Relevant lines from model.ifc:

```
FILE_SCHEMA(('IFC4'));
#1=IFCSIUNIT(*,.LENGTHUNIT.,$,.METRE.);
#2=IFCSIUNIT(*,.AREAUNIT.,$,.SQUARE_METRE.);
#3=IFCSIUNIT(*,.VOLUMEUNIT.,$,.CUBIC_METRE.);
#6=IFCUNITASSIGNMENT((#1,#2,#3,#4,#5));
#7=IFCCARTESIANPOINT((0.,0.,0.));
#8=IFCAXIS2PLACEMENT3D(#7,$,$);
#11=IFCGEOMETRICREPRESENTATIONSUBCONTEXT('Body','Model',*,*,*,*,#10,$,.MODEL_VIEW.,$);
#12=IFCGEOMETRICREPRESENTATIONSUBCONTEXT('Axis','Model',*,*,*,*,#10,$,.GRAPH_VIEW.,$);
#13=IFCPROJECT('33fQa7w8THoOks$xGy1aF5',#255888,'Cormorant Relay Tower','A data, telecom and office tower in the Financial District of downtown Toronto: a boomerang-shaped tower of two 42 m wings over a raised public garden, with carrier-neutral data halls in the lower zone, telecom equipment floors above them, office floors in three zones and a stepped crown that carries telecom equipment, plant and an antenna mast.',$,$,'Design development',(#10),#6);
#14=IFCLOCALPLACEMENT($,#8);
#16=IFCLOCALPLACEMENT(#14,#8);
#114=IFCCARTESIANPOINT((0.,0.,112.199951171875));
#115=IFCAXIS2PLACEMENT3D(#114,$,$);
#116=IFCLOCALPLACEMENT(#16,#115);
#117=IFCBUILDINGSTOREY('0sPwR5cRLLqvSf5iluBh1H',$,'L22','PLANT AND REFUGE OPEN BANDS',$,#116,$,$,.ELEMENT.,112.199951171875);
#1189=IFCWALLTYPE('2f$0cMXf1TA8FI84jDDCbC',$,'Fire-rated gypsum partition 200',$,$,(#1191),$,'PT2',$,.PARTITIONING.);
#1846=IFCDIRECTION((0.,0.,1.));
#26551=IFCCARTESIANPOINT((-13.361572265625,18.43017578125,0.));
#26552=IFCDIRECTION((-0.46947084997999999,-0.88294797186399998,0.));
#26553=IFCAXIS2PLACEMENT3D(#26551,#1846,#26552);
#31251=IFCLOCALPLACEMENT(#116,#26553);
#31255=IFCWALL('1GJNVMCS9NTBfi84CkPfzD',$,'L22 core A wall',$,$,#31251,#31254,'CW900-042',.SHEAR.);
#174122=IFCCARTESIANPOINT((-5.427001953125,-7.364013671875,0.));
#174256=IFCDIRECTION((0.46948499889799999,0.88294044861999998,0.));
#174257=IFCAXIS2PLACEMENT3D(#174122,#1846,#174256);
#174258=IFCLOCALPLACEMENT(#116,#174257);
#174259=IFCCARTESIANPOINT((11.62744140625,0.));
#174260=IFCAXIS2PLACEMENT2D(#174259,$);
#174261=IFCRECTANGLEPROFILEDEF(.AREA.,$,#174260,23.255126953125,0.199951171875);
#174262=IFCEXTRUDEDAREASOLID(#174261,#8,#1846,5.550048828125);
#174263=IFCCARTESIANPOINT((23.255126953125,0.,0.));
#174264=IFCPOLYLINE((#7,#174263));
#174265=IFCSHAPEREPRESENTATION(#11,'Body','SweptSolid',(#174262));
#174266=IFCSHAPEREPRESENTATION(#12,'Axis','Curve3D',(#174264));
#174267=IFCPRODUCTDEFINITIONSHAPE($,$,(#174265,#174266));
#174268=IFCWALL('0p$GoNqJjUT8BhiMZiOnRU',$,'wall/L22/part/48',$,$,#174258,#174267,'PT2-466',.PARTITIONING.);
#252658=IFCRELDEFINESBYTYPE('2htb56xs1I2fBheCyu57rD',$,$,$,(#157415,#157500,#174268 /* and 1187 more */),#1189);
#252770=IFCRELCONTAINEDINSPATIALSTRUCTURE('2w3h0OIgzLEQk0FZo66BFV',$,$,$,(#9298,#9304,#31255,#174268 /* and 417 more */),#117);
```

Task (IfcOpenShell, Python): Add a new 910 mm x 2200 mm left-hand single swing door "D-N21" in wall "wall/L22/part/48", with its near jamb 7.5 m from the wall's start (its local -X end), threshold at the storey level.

```python
import numpy as np
import ifcopenshell
import ifcopenshell.api.feature
import ifcopenshell.api.geometry
import ifcopenshell.api.root
import ifcopenshell.api.spatial
import ifcopenshell.geom
import ifcopenshell.util.element
import ifcopenshell.util.placement
import ifcopenshell.util.representation
import ifcopenshell.util.shape
import ifcopenshell.util.unit

model = ifcopenshell.open("model.ifc")
unit_scale = ifcopenshell.util.unit.calculate_unit_scale(model)
settings = ifcopenshell.geom.settings()


def volume(element):
    """Net volume in cubic metres, openings subtracted."""
    shape = ifcopenshell.geom.create_shape(settings, element)
    return ifcopenshell.util.shape.get_volume(shape.geometry)


wall = model.by_id(174268)
storey = ifcopenshell.util.element.get_container(wall, ifc_class="IfcBuildingStorey")
context = ifcopenshell.util.representation.get_context(model, "Model", "Body", "MODEL_VIEW")
before = volume(wall)

width, height, from_end, sill = 0.91, 2.2, 7.5, 0.0  # metres

# The wall runs along its own X axis, and the end named is its -X end.
wall_shape = ifcopenshell.geom.create_shape(settings, wall)
x, y, z = ifcopenshell.util.shape.get_vertices(wall_shape.geometry).T
start = x.min() + from_end
face, thickness = float(y.min()), float(y.max() - y.min())
wall_matrix = ifcopenshell.util.placement.get_local_placement(wall.ObjectPlacement)
level = ifcopenshell.util.placement.get_local_placement(storey.ObjectPlacement)[2, 3]


def in_wall(x, y):
    """Placement at x, y metres in the wall's axes, at sill height."""
    matrix = wall_matrix.copy()
    matrix[:, 3] = wall_matrix @ np.array([x / unit_scale, y / unit_scale, 0.0, 1.0])
    matrix[2, 3] = level + sill / unit_scale
    return matrix


# Opening: a box that overshoots both wall faces by 50 mm.
opening = ifcopenshell.api.root.create_entity(model, ifc_class="IfcOpeningElement", predefined_type="OPENING")
box = ifcopenshell.api.geometry.add_wall_representation(
    model, context=context, length=width, height=height, thickness=thickness + 0.1
)
ifcopenshell.api.geometry.assign_representation(model, product=opening, representation=box)
ifcopenshell.api.geometry.edit_object_placement(model, product=opening, matrix=in_wall(start, face - 0.05), is_si=False)
ifcopenshell.api.feature.add_feature(model, feature=opening, element=wall)

door = ifcopenshell.api.root.create_entity(model, ifc_class="IfcDoor", name="D-N21", predefined_type="DOOR")
door.OverallWidth, door.OverallHeight = width / unit_scale, height / unit_scale
door.OperationType = "SINGLE_SWING_LEFT"
body = ifcopenshell.api.geometry.add_door_representation(
    model,
    context=context,
    overall_width=door.OverallWidth,
    overall_height=door.OverallHeight,
    operation_type="SINGLE_SWING_LEFT",
    lining_properties={"LiningDepth": thickness / unit_scale, "ThresholdDepth": thickness / unit_scale},
)
ifcopenshell.api.geometry.assign_representation(model, product=door, representation=body)
ifcopenshell.api.spatial.assign_container(model, products=[door], relating_structure=storey)
ifcopenshell.api.feature.add_filling(model, opening=opening, element=door)

# The lining spans the wall, so the door starts at the wall face.
ifcopenshell.api.geometry.edit_object_placement(model, product=door, matrix=in_wall(start, face), is_si=False)

after = volume(wall)

print(f"wall volume {before:.3f} -> {after:.3f} m3")

model.write("model-out.ifc")
```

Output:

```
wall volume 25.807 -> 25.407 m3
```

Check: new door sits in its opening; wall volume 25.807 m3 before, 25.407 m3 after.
